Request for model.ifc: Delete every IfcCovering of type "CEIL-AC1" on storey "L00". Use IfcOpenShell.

First a look at what the model holds.

```python
import ifcopenshell
import ifcopenshell.util.element

model = ifcopenshell.open("model.ifc")
print(model.schema)
storey = next(s for s in model.by_type("IfcBuildingStorey") if s.Name == "L00")
coverings = [e for e in ifcopenshell.util.element.get_decomposition(storey) if e.is_a("IfcCovering")]
seen = {}
for e in coverings:
    element_type = ifcopenshell.util.element.get_type(e)
    name = element_type.Name if element_type not in (None, e) else None
    seen[name] = seen.get(name, 0) + 1
for name, count in sorted(seen.items(), key=str):
    print(count, "x", name)
```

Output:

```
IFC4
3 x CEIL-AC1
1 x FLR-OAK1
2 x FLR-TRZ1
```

```python
import ifcopenshell
import ifcopenshell.api.root
import ifcopenshell.util.element

model = ifcopenshell.open("model.ifc")

storey = next(s for s in model.by_type("IfcBuildingStorey") if s.Name == "L00")
coverings = [e for e in ifcopenshell.util.element.get_decomposition(storey) if e.is_a("IfcCovering")]
targets = [e for e in coverings if (t := ifcopenshell.util.element.get_type(e)) not in (None, e) and t.Name == "CEIL-AC1"]

for e in targets:
    ifcopenshell.api.root.remove_product(model, product=e)
print(len(targets), "removed")

model.write("model-out.ifc")
```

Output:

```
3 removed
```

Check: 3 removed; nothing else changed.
